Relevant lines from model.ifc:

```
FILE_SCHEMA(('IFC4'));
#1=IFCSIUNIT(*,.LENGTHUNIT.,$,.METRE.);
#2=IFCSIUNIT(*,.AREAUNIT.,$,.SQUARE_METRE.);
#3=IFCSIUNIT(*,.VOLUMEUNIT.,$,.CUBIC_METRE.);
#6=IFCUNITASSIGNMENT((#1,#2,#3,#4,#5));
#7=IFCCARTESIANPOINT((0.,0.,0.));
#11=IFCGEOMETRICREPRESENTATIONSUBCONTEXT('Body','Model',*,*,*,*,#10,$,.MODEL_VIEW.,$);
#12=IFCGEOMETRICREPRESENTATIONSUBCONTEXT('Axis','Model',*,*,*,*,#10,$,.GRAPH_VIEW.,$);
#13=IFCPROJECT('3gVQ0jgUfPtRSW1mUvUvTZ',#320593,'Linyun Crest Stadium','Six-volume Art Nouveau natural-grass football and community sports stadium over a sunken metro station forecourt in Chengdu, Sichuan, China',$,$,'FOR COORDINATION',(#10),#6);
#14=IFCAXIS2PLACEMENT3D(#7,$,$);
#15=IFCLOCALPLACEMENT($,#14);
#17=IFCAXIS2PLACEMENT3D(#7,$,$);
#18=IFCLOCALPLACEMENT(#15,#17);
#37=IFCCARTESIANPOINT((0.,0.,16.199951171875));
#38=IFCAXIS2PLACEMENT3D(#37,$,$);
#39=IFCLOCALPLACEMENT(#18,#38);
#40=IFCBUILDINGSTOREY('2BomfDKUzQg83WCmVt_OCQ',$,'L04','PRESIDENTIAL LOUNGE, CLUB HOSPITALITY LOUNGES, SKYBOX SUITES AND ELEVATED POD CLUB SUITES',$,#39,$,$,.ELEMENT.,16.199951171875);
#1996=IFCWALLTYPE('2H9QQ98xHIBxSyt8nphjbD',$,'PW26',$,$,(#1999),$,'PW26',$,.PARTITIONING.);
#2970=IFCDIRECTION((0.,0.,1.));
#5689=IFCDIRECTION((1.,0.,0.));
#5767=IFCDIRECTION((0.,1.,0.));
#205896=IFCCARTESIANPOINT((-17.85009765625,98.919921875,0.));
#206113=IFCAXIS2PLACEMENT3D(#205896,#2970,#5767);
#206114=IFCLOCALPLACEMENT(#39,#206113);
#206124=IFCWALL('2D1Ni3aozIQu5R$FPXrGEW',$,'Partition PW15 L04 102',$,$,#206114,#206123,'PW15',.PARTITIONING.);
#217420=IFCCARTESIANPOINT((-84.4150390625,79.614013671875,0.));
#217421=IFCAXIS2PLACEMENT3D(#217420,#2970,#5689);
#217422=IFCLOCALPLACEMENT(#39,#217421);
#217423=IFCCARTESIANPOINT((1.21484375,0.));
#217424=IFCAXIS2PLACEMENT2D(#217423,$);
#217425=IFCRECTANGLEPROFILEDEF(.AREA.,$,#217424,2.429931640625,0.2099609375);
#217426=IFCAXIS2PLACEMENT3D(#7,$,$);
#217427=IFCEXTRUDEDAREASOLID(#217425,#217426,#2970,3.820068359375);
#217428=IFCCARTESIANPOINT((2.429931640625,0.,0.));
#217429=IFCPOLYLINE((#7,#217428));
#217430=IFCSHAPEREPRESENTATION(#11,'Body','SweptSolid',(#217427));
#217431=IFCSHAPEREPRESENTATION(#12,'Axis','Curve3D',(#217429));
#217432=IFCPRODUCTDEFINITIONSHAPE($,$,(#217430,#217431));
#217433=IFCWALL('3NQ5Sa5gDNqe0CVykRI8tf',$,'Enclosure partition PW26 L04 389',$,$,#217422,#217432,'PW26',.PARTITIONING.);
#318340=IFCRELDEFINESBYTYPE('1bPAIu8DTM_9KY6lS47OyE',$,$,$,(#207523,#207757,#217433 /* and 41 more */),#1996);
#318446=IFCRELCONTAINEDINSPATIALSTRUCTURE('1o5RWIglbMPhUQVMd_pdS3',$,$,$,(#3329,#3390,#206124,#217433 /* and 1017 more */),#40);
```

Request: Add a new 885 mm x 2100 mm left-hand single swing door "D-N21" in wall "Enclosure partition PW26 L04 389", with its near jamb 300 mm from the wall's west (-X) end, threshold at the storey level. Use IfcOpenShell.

```python
import numpy as np
import ifcopenshell
import ifcopenshell.api.feature
import ifcopenshell.api.geometry
import ifcopenshell.api.root
import ifcopenshell.api.spatial
import ifcopenshell.geom
import ifcopenshell.util.element
import ifcopenshell.util.placement
import ifcopenshell.util.representation
import ifcopenshell.util.shape
import ifcopenshell.util.unit

model = ifcopenshell.open("model.ifc")
unit_scale = ifcopenshell.util.unit.calculate_unit_scale(model)
settings = ifcopenshell.geom.settings()


def volume(element):
    """Net volume in cubic metres, openings subtracted."""
    shape = ifcopenshell.geom.create_shape(settings, element)
    return ifcopenshell.util.shape.get_volume(shape.geometry)


wall = model.by_id(217433)
storey = ifcopenshell.util.element.get_container(wall, ifc_class="IfcBuildingStorey")
context = ifcopenshell.util.representation.get_context(model, "Model", "Body", "MODEL_VIEW")
before = volume(wall)

width, height, from_end, sill = 0.885, 2.1, 0.3, 0.0  # metres

# The wall runs along its own X axis, and the end named is its -X end.
wall_shape = ifcopenshell.geom.create_shape(settings, wall)
x, y, z = ifcopenshell.util.shape.get_vertices(wall_shape.geometry).T
start = x.min() + from_end
face, thickness = float(y.min()), float(y.max() - y.min())
wall_matrix = ifcopenshell.util.placement.get_local_placement(wall.ObjectPlacement)
level = ifcopenshell.util.placement.get_local_placement(storey.ObjectPlacement)[2, 3]


def in_wall(x, y):
    """Placement at x, y metres in the wall's axes, at sill height."""
    matrix = wall_matrix.copy()
    matrix[:, 3] = wall_matrix @ np.array([x / unit_scale, y / unit_scale, 0.0, 1.0])
    matrix[2, 3] = level + sill / unit_scale
    return matrix


# Opening: a box that overshoots both wall faces by 50 mm.
opening = ifcopenshell.api.root.create_entity(model, ifc_class="IfcOpeningElement", predefined_type="OPENING")
box = ifcopenshell.api.geometry.add_wall_representation(
    model, context=context, length=width, height=height, thickness=thickness + 0.1
)
ifcopenshell.api.geometry.assign_representation(model, product=opening, representation=box)
ifcopenshell.api.geometry.edit_object_placement(model, product=opening, matrix=in_wall(start, face - 0.05), is_si=False)
ifcopenshell.api.feature.add_feature(model, feature=opening, element=wall)

door = ifcopenshell.api.root.create_entity(model, ifc_class="IfcDoor", name="D-N21", predefined_type="DOOR")
door.OverallWidth, door.OverallHeight = width / unit_scale, height / unit_scale
door.OperationType = "SINGLE_SWING_LEFT"
body = ifcopenshell.api.geometry.add_door_representation(
    model,
    context=context,
    overall_width=door.OverallWidth,
    overall_height=door.OverallHeight,
    operation_type="SINGLE_SWING_LEFT",
    lining_properties={"LiningDepth": thickness / unit_scale, "ThresholdDepth": thickness / unit_scale},
)
ifcopenshell.api.geometry.assign_representation(model, product=door, representation=body)
ifcopenshell.api.spatial.assign_container(model, products=[door], relating_structure=storey)
ifcopenshell.api.feature.add_filling(model, opening=opening, element=door)

# The lining spans the wall, so the door starts at the wall face.
ifcopenshell.api.geometry.edit_object_placement(model, product=door, matrix=in_wall(start, face), is_si=False)

after = volume(wall)

print(f"wall volume {before:.3f} -> {after:.3f} m3")

model.write("model_updated.ifc")
```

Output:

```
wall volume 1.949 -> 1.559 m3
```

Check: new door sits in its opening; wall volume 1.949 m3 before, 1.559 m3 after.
